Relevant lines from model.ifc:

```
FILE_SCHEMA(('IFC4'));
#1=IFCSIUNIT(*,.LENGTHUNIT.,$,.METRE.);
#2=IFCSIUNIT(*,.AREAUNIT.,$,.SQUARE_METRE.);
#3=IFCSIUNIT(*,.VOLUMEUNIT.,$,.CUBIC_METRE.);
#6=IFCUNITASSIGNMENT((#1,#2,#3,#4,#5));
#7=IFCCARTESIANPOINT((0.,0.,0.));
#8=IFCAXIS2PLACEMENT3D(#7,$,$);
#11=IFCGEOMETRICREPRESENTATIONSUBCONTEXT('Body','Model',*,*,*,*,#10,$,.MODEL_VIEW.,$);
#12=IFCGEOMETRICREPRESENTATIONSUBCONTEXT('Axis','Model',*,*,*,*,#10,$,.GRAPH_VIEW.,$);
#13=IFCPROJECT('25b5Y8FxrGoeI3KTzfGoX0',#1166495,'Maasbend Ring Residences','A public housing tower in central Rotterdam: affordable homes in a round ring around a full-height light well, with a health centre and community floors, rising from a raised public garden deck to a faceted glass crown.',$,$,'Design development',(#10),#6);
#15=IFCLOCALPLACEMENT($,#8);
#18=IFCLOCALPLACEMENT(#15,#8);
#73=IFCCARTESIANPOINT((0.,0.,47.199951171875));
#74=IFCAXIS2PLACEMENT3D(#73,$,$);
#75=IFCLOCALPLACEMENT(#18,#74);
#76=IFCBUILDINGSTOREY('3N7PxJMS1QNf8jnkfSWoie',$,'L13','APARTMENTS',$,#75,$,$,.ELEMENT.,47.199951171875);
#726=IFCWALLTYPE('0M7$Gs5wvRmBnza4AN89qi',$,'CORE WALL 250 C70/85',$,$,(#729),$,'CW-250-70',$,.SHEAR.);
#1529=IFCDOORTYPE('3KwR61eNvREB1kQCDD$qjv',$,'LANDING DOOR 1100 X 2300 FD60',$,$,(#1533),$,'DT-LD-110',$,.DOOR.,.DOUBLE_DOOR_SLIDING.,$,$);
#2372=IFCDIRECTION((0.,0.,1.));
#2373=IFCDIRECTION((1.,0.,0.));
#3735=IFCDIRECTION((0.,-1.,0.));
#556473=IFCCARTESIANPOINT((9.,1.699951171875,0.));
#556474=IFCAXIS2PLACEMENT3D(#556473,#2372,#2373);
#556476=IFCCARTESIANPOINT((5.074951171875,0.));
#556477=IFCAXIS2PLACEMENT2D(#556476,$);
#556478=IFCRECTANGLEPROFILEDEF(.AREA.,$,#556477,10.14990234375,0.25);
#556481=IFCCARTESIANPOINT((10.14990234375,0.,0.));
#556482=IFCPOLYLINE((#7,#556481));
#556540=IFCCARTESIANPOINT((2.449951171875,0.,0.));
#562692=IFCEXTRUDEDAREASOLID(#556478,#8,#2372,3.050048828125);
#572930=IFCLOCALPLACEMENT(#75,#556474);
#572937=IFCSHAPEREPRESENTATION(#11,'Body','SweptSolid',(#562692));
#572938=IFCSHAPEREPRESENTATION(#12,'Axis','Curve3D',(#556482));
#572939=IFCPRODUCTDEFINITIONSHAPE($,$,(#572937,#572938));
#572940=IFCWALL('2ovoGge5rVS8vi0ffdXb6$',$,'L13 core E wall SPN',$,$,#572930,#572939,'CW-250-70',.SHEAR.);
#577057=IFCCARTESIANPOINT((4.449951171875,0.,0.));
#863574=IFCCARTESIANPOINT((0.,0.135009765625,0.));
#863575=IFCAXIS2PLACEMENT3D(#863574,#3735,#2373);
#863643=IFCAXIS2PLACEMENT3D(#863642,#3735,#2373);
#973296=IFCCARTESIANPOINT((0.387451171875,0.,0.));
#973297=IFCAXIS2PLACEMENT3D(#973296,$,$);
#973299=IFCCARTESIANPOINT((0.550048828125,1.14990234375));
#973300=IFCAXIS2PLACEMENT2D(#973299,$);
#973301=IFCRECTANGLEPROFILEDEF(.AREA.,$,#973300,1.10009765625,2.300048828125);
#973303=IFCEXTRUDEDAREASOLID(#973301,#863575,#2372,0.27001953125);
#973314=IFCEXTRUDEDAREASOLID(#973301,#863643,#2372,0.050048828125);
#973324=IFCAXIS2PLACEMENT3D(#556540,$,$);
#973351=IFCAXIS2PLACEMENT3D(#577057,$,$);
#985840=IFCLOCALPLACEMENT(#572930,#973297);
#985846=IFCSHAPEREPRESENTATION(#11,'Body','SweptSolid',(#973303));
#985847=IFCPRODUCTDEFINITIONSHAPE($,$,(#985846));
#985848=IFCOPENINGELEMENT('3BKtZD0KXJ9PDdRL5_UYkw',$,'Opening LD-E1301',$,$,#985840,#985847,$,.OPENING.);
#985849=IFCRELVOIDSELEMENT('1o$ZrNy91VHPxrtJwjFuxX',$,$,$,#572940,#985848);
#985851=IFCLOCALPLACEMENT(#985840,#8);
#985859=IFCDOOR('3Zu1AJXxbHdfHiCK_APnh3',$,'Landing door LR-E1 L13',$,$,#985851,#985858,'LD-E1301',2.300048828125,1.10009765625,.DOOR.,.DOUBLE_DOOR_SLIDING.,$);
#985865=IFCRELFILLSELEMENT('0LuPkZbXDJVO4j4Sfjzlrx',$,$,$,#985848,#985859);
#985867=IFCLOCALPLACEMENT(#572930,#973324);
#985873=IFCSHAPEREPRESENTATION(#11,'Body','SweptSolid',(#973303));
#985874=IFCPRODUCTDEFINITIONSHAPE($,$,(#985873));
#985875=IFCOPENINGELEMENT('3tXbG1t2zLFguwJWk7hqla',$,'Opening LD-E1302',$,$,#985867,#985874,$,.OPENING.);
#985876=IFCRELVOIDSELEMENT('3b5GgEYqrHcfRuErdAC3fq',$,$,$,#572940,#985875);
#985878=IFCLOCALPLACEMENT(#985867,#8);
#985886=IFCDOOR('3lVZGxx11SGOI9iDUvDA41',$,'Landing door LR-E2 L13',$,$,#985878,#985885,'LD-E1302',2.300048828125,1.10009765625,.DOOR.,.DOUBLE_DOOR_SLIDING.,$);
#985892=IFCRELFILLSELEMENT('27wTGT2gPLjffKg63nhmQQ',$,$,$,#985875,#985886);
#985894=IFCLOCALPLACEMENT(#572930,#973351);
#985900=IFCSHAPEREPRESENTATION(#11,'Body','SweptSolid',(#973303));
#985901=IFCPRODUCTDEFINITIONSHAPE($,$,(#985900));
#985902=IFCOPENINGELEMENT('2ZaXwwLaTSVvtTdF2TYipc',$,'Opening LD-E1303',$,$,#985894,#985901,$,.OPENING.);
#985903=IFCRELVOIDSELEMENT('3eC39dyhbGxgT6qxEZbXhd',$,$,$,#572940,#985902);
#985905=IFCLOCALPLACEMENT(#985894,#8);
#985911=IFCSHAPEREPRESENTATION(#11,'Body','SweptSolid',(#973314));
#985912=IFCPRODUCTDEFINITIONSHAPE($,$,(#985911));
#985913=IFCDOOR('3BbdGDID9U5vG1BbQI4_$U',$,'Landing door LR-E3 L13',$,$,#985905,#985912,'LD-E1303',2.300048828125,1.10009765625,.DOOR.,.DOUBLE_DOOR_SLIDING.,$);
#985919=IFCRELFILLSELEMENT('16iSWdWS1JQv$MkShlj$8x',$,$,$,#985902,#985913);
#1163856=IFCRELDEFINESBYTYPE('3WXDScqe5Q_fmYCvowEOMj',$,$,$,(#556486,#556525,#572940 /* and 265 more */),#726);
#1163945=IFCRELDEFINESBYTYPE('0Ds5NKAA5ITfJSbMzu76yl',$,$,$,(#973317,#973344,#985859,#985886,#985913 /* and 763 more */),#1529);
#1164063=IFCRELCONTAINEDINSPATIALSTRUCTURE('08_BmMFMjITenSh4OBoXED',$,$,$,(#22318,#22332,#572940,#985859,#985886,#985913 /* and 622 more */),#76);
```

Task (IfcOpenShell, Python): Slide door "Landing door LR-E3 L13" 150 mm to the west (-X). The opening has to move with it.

```python
import ifcopenshell
import ifcopenshell.api.geometry
import ifcopenshell.util.placement

model = ifcopenshell.open("model.ifc")

door = model.by_guid("3BbdGDID9U5vG1BbQI4_$U")
opening = door.FillsVoids[0].RelatingOpeningElement
wall = opening.VoidsElements[0].RelatingBuildingElement

wall_matrix = ifcopenshell.util.placement.get_local_placement(wall.ObjectPlacement)
shift = wall_matrix[:3, 0] * -0.15
before = ifcopenshell.util.placement.get_local_placement(door.ObjectPlacement)[:3, 3].copy()

# The door is placed relative to its opening, so it follows when the opening moves.
matrix = ifcopenshell.util.placement.get_local_placement(opening.ObjectPlacement)
matrix[:3, 3] += shift
ifcopenshell.api.geometry.edit_object_placement(
    model, product=opening, matrix=matrix, is_si=False, should_transform_children=True
)

after = ifcopenshell.util.placement.get_local_placement(door.ObjectPlacement)[:3, 3]
print("door moved by", (after - before).round(3) + 0.0)

model.write("model_v2.ifc")
```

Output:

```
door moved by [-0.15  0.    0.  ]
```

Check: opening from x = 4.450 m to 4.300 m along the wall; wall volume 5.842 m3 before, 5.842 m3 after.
